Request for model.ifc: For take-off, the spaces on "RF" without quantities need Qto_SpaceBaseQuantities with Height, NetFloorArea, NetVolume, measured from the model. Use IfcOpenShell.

First a look at what the model holds.

```python
import ifcopenshell
import ifcopenshell.util.element
import ifcopenshell.util.unit

model = ifcopenshell.open("model.ifc")
print(model.schema)
for unit_type in ("LENGTHUNIT", "AREAUNIT", "VOLUMEUNIT"):
    print(unit_type, ifcopenshell.util.unit.calculate_unit_scale(model, unit_type))
storey = next(s for s in model.by_type("IfcBuildingStorey") if s.Name == "RF")
spaces = [e for e in ifcopenshell.util.element.get_decomposition(storey) if e.is_a("IfcSpace")]
for e in sorted(spaces, key=lambda e: e.id()):
    print(e.id(), e.is_a(), e.Name, list(ifcopenshell.util.element.get_psets(e, qtos_only=True)), sep=" | ")
```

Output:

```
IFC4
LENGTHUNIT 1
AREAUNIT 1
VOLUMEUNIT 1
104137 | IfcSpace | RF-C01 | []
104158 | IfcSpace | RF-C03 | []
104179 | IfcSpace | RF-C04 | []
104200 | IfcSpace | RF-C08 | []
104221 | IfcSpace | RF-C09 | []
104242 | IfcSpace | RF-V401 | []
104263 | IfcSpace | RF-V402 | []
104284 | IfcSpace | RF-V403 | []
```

```python
import ifcopenshell
import ifcopenshell.api.pset
import ifcopenshell.geom
import ifcopenshell.util.element
import ifcopenshell.util.shape
import ifcopenshell.util.unit

model = ifcopenshell.open("model.ifc")
unit_scale = ifcopenshell.util.unit.calculate_unit_scale(model)
area_scale = ifcopenshell.util.unit.calculate_unit_scale(model, "AREAUNIT")
volume_scale = ifcopenshell.util.unit.calculate_unit_scale(model, "VOLUMEUNIT")
settings = ifcopenshell.geom.settings()

storey = next(s for s in model.by_type("IfcBuildingStorey") if s.Name == "RF")
spaces = [e for e in ifcopenshell.util.element.get_decomposition(storey) if e.is_a("IfcSpace")]

for e in sorted(spaces, key=lambda e: e.id()):
    if ifcopenshell.util.element.get_psets(e, qtos_only=True, should_inherit=False):
        continue
    # Geometry comes back in metres, in the element's own axes.
    shape = ifcopenshell.geom.create_shape(settings, e)
    values = {
        "Height": ifcopenshell.util.shape.get_z(shape.geometry) / unit_scale,
        "NetFloorArea": ifcopenshell.util.shape.get_footprint_area(shape.geometry) / area_scale,
        "NetVolume": ifcopenshell.util.shape.get_volume(shape.geometry) / volume_scale,
    }
    qto = ifcopenshell.api.pset.add_qto(model, product=e, name="Qto_SpaceBaseQuantities")
    ifcopenshell.api.pset.edit_qto(model, qto=qto, properties=values)
    print(e.id(), {k: round(v, 3) for k, v in values.items()})

model.write("model_updated.ifc")
```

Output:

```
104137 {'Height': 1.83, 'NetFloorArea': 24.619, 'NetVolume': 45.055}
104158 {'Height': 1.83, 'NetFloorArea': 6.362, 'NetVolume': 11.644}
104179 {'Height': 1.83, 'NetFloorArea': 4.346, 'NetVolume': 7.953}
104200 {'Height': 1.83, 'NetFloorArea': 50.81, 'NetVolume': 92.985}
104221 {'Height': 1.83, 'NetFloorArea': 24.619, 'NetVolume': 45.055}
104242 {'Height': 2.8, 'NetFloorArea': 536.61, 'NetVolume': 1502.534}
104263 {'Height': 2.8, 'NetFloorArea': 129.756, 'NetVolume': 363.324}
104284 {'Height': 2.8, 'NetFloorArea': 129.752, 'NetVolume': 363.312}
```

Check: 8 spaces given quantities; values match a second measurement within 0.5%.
